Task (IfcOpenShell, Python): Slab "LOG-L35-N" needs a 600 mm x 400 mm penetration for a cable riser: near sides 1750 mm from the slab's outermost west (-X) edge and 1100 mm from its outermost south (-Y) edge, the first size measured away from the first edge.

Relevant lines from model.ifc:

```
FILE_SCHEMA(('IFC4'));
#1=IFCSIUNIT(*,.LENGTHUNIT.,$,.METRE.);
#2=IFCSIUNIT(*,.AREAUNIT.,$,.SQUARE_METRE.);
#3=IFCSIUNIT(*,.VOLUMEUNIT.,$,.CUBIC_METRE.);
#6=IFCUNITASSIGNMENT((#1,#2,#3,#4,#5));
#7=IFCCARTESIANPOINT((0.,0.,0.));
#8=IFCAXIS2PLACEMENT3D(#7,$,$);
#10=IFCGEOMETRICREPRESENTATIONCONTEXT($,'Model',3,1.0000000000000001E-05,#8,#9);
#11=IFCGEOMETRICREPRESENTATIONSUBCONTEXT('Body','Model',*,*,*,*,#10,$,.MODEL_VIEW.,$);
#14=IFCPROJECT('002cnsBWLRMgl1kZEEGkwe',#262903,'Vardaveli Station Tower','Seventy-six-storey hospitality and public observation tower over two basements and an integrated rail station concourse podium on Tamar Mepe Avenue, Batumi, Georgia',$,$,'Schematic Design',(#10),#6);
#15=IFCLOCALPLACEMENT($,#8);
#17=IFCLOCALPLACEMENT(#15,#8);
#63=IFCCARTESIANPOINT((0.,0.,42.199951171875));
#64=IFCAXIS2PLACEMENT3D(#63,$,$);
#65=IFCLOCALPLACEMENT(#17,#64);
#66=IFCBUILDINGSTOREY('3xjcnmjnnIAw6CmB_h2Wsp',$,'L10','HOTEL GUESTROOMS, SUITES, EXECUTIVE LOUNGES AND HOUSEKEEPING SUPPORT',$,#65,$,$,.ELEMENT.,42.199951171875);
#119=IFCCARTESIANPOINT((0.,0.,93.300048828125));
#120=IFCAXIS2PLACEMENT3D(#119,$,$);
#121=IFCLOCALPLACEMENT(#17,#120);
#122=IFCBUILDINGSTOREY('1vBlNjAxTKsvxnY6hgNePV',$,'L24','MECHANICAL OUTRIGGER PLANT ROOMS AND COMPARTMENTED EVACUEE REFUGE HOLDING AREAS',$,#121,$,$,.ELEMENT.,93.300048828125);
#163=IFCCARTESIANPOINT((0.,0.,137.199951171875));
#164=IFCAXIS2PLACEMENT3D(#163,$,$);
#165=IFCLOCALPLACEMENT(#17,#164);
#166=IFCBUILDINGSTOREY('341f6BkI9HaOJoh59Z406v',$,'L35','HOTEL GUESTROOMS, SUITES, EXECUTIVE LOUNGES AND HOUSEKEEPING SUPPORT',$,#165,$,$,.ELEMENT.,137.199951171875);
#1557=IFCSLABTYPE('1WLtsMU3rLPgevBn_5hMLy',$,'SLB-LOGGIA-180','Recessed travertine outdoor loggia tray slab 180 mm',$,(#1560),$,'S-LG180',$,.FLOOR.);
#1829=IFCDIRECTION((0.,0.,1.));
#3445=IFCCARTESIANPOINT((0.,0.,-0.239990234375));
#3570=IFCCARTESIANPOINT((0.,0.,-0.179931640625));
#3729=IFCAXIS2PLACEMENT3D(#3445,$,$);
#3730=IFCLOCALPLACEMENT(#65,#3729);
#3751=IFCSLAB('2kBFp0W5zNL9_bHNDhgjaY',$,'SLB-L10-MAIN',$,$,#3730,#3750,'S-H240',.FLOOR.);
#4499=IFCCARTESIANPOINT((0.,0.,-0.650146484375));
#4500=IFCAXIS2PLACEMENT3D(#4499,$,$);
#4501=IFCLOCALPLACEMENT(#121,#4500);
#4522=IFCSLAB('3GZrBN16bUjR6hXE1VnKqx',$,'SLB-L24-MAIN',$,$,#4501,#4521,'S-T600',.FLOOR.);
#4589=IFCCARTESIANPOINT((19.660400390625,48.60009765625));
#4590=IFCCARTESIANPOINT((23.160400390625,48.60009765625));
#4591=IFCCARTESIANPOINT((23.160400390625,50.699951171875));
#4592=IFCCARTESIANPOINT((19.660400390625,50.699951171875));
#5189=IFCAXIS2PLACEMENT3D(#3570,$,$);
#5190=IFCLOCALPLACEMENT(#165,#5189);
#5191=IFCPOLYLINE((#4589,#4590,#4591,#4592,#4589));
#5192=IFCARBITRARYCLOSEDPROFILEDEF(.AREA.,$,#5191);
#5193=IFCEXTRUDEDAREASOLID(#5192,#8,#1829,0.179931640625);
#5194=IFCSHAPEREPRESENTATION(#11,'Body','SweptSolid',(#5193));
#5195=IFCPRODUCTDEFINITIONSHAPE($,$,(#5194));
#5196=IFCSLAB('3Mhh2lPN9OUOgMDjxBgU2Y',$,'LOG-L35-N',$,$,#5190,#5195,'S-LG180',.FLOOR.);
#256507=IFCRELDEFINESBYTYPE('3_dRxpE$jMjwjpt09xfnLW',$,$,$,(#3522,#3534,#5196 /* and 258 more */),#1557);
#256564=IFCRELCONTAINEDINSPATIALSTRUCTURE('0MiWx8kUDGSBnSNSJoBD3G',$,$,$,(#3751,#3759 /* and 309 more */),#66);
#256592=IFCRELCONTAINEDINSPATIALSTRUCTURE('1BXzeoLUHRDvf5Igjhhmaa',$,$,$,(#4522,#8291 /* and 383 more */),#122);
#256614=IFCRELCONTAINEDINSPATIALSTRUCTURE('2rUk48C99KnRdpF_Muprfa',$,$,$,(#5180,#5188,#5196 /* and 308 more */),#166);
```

```python
import numpy as np
import ifcopenshell
import ifcopenshell.api.feature
import ifcopenshell.api.geometry
import ifcopenshell.api.root
import ifcopenshell.geom
import ifcopenshell.util.placement
import ifcopenshell.util.representation
import ifcopenshell.util.shape
import ifcopenshell.util.unit

model = ifcopenshell.open("model.ifc")
unit_scale = ifcopenshell.util.unit.calculate_unit_scale(model)
settings = ifcopenshell.geom.settings()


def volume(element):
    """Net volume in cubic metres, openings subtracted."""
    shape = ifcopenshell.geom.create_shape(settings, element)
    return ifcopenshell.util.shape.get_volume(shape.geometry)


slab = model.by_guid("3Mhh2lPN9OUOgMDjxBgU2Y")
before = volume(slab)

# Extent in the slab's own axes, in metres. The edges named are its -X and -Y sides.
slab_shape = ifcopenshell.geom.create_shape(settings, slab)
vertices = ifcopenshell.util.shape.get_vertices(slab_shape.geometry)
x_min, y_min, bottom = vertices.min(axis=0)
top = vertices[:, 2].max()

opening = ifcopenshell.api.root.create_entity(model, ifc_class="IfcOpeningElement", name="Cable riser opening", predefined_type="OPENING")
context = ifcopenshell.util.representation.get_context(model, "Model", "Body", "MODEL_VIEW")
width, depth = 0.6, 0.4
outline = [(0.0, 0.0), (width, 0.0), (width, depth), (0.0, depth), (0.0, 0.0)]
# Overshoot both faces by 50 mm so the cut is clean.
shape = ifcopenshell.api.geometry.add_slab_representation(
    model, context=context, depth=top - bottom + 0.1, polyline=outline
)
ifcopenshell.api.geometry.assign_representation(model, product=opening, representation=shape)

matrix = ifcopenshell.util.placement.get_local_placement(slab.ObjectPlacement)
matrix[:, 3] = matrix @ np.append(np.array([x_min + 1.75, y_min + 1.1, bottom - 0.05]) / unit_scale, 1.0)
ifcopenshell.api.geometry.edit_object_placement(model, product=opening, matrix=matrix, is_si=False)
ifcopenshell.api.feature.add_feature(model, feature=opening, element=slab)

after = volume(slab)

print(f"slab volume {before:.3f} -> {after:.3f} m3")

model.write("model_rev.ifc")
```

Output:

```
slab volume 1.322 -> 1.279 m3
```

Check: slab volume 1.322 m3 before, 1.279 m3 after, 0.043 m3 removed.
